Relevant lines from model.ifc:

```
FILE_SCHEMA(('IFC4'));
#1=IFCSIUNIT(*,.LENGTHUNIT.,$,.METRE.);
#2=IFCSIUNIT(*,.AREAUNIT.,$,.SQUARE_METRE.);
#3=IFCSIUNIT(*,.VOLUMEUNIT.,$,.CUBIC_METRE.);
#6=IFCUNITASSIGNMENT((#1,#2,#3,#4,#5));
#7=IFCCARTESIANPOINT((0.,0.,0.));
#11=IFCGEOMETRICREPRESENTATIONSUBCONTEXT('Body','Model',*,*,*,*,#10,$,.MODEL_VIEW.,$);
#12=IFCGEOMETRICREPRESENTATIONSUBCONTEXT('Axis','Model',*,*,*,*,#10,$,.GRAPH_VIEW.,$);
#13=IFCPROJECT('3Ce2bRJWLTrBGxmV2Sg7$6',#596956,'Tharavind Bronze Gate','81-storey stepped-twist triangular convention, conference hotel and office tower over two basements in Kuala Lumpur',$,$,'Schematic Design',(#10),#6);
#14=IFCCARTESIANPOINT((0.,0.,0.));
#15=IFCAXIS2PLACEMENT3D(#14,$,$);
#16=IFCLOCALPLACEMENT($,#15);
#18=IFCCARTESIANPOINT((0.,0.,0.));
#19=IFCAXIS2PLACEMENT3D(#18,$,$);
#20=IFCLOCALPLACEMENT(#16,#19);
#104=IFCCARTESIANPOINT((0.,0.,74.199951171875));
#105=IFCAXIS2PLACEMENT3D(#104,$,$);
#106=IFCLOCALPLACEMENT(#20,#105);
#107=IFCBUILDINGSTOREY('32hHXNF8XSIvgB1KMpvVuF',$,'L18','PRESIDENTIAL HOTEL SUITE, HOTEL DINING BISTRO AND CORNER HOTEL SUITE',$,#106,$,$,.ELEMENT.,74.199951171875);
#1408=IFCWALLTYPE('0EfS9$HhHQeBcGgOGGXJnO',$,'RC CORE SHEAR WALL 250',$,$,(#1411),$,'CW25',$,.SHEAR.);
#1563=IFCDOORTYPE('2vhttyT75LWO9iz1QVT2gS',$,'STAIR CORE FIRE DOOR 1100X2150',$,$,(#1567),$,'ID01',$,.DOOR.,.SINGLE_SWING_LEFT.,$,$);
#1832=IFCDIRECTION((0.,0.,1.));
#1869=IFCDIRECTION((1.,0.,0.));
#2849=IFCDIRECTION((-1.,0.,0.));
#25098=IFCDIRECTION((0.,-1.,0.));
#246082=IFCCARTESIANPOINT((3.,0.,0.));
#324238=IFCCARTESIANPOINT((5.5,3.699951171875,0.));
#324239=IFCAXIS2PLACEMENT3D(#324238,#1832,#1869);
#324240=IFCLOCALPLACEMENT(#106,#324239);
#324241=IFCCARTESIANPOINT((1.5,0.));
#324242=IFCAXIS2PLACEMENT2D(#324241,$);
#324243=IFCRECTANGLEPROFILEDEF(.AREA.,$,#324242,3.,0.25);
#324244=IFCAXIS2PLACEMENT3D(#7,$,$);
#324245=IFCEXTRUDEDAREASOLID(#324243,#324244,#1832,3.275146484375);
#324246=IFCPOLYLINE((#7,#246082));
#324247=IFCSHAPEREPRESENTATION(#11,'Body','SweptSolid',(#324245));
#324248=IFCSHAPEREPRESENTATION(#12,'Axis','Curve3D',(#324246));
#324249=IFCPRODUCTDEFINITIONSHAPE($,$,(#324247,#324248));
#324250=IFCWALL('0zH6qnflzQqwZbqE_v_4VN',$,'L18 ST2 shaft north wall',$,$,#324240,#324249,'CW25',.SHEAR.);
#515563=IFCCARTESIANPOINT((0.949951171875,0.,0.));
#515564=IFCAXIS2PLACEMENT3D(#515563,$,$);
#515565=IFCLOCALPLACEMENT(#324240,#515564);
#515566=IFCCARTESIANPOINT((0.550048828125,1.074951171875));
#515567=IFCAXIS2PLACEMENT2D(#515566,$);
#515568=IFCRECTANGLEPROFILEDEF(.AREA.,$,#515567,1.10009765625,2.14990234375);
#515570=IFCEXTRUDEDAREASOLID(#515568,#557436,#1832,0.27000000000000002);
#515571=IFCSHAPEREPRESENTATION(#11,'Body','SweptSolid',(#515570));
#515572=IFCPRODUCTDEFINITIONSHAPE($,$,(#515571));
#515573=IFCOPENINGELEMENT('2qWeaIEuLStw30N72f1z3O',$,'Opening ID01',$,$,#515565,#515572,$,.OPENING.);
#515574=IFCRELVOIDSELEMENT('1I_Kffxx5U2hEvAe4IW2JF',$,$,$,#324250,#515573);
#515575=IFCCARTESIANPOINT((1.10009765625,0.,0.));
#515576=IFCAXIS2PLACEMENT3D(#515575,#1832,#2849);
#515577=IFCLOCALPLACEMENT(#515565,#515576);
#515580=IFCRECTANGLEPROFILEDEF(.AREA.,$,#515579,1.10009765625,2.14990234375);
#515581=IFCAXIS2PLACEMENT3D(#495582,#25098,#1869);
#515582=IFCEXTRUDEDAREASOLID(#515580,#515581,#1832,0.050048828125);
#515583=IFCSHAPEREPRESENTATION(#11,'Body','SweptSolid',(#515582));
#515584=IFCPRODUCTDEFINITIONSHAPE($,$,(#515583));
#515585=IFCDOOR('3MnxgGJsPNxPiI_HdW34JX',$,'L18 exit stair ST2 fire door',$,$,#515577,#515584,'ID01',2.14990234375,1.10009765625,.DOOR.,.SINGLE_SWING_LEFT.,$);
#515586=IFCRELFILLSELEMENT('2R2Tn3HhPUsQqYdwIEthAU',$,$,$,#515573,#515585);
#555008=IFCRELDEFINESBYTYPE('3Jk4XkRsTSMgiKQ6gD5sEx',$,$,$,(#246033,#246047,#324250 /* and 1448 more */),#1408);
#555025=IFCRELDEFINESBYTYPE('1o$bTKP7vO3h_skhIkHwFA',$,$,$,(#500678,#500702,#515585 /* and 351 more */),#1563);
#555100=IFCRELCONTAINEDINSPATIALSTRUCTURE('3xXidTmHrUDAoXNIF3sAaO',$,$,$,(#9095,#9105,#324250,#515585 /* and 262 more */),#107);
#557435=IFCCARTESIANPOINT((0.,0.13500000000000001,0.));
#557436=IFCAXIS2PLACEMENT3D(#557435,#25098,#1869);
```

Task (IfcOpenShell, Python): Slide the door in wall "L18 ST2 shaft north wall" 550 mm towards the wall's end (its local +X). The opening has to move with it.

```python
import ifcopenshell
import ifcopenshell.api.geometry
import ifcopenshell.util.placement
import ifcopenshell.util.unit

model = ifcopenshell.open("model.ifc")
unit_scale = ifcopenshell.util.unit.calculate_unit_scale(model)

door = model.by_guid("3MnxgGJsPNxPiI_HdW34JX")
opening = door.FillsVoids[0].RelatingOpeningElement
wall = opening.VoidsElements[0].RelatingBuildingElement

wall_matrix = ifcopenshell.util.placement.get_local_placement(wall.ObjectPlacement)
shift = wall_matrix[:3, 0] * 0.55 / unit_scale
before = ifcopenshell.util.placement.get_local_placement(door.ObjectPlacement)[:3, 3].copy()

# The door is placed relative to its opening, so it follows when the opening moves.
matrix = ifcopenshell.util.placement.get_local_placement(opening.ObjectPlacement)
matrix[:3, 3] += shift
ifcopenshell.api.geometry.edit_object_placement(
    model, product=opening, matrix=matrix, is_si=False, should_transform_children=True
)

after = ifcopenshell.util.placement.get_local_placement(door.ObjectPlacement)[:3, 3]
print("door moved by", (after - before).round(3) + 0.0)

model.write("model-out.ifc")
```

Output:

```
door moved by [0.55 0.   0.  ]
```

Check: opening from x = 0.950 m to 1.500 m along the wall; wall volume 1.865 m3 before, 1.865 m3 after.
